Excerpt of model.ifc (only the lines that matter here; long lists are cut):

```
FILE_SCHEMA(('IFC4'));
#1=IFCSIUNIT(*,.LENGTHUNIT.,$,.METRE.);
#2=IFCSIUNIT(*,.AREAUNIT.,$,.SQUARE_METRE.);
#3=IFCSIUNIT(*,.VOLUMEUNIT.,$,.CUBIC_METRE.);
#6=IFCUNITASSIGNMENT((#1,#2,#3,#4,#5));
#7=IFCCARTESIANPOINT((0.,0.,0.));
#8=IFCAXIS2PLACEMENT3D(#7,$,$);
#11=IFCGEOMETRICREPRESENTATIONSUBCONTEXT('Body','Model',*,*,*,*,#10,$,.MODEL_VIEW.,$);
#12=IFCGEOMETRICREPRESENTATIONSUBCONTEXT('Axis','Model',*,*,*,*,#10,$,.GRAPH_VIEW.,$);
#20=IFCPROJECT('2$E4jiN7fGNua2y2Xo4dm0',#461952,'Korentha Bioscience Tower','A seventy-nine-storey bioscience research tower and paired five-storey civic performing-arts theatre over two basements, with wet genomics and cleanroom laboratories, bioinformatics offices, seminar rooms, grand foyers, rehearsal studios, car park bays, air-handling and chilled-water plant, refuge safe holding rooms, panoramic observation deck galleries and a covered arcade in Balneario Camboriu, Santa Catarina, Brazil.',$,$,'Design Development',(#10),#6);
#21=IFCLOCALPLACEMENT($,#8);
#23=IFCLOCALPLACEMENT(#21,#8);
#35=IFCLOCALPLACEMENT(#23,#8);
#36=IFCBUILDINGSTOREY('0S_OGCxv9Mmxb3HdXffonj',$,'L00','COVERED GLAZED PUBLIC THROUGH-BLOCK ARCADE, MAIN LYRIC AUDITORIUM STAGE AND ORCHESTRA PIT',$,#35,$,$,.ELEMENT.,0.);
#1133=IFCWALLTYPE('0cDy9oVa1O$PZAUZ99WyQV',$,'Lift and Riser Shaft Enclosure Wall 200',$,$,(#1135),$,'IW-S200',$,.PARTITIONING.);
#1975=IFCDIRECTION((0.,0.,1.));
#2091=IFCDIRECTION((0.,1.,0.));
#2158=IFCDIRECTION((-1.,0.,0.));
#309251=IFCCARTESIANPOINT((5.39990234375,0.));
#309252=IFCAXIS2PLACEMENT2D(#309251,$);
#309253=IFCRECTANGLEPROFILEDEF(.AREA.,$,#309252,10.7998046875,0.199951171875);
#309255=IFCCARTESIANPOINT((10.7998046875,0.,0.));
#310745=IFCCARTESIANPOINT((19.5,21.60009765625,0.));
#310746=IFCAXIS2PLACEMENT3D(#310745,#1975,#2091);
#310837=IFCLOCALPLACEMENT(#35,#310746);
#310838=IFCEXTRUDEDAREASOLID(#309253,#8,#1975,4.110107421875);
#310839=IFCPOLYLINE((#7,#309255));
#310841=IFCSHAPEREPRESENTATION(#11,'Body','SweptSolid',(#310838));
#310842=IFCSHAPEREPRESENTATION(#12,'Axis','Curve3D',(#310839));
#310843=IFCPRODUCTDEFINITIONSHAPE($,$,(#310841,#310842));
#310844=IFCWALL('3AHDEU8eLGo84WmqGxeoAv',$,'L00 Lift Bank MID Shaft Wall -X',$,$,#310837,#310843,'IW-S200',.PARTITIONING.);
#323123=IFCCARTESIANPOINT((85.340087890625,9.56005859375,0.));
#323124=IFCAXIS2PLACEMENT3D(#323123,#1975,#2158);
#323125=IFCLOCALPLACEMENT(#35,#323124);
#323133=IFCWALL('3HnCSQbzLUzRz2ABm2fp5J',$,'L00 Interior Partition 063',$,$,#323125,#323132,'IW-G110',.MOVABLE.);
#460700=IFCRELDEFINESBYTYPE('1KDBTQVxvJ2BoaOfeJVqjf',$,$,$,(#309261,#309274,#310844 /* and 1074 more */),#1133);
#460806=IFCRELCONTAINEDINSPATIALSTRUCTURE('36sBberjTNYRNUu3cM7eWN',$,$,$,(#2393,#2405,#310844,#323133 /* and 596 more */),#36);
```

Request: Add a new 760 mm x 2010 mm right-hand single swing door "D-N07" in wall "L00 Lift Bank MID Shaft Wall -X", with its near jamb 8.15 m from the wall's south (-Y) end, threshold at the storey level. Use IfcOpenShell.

```python
import numpy as np
import ifcopenshell
import ifcopenshell.api.feature
import ifcopenshell.api.geometry
import ifcopenshell.api.root
import ifcopenshell.api.spatial
import ifcopenshell.geom
import ifcopenshell.util.element
import ifcopenshell.util.placement
import ifcopenshell.util.representation
import ifcopenshell.util.shape
import ifcopenshell.util.unit

model = ifcopenshell.open("model.ifc")
unit_scale = ifcopenshell.util.unit.calculate_unit_scale(model)
settings = ifcopenshell.geom.settings()


def volume(element):
    """Net volume in cubic metres, openings subtracted."""
    shape = ifcopenshell.geom.create_shape(settings, element)
    return ifcopenshell.util.shape.get_volume(shape.geometry)


wall = model.by_guid("3AHDEU8eLGo84WmqGxeoAv")
storey = ifcopenshell.util.element.get_container(wall, ifc_class="IfcBuildingStorey")
context = ifcopenshell.util.representation.get_context(model, "Model", "Body", "MODEL_VIEW")
before = volume(wall)

width, height, from_end, sill = 0.76, 2.01, 8.15, 0.0  # metres

# The wall runs along its own X axis, and the end named is its -X end.
wall_shape = ifcopenshell.geom.create_shape(settings, wall)
x, y, z = ifcopenshell.util.shape.get_vertices(wall_shape.geometry).T
start = x.min() + from_end
face, thickness = float(y.min()), float(y.max() - y.min())
wall_matrix = ifcopenshell.util.placement.get_local_placement(wall.ObjectPlacement)
level = ifcopenshell.util.placement.get_local_placement(storey.ObjectPlacement)[2, 3]


def in_wall(x, y):
    """Placement at x, y metres in the wall's axes, at sill height."""
    matrix = wall_matrix.copy()
    matrix[:, 3] = wall_matrix @ np.array([x / unit_scale, y / unit_scale, 0.0, 1.0])
    matrix[2, 3] = level + sill / unit_scale
    return matrix


# Opening: a box that overshoots both wall faces by 50 mm.
opening = ifcopenshell.api.root.create_entity(model, ifc_class="IfcOpeningElement", predefined_type="OPENING")
box = ifcopenshell.api.geometry.add_wall_representation(
    model, context=context, length=width, height=height, thickness=thickness + 0.1
)
ifcopenshell.api.geometry.assign_representation(model, product=opening, representation=box)
ifcopenshell.api.geometry.edit_object_placement(model, product=opening, matrix=in_wall(start, face - 0.05), is_si=False)
ifcopenshell.api.feature.add_feature(model, feature=opening, element=wall)

door = ifcopenshell.api.root.create_entity(model, ifc_class="IfcDoor", name="D-N07", predefined_type="DOOR")
door.OverallWidth, door.OverallHeight = width / unit_scale, height / unit_scale
door.OperationType = "SINGLE_SWING_RIGHT"
body = ifcopenshell.api.geometry.add_door_representation(
    model,
    context=context,
    overall_width=door.OverallWidth,
    overall_height=door.OverallHeight,
    operation_type="SINGLE_SWING_RIGHT",
    lining_properties={"LiningDepth": thickness / unit_scale, "ThresholdDepth": thickness / unit_scale},
)
ifcopenshell.api.geometry.assign_representation(model, product=door, representation=body)
ifcopenshell.api.spatial.assign_container(model, products=[door], relating_structure=storey)
ifcopenshell.api.feature.add_filling(model, opening=opening, element=door)

# The lining spans the wall, so the door starts at the wall face.
ifcopenshell.api.geometry.edit_object_placement(model, product=door, matrix=in_wall(start, face), is_si=False)

after = volume(wall)

print(f"wall volume {before:.3f} -> {after:.3f} m3")

model.write("model-out.ifc")
```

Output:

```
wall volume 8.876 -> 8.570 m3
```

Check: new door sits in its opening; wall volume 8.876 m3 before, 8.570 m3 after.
